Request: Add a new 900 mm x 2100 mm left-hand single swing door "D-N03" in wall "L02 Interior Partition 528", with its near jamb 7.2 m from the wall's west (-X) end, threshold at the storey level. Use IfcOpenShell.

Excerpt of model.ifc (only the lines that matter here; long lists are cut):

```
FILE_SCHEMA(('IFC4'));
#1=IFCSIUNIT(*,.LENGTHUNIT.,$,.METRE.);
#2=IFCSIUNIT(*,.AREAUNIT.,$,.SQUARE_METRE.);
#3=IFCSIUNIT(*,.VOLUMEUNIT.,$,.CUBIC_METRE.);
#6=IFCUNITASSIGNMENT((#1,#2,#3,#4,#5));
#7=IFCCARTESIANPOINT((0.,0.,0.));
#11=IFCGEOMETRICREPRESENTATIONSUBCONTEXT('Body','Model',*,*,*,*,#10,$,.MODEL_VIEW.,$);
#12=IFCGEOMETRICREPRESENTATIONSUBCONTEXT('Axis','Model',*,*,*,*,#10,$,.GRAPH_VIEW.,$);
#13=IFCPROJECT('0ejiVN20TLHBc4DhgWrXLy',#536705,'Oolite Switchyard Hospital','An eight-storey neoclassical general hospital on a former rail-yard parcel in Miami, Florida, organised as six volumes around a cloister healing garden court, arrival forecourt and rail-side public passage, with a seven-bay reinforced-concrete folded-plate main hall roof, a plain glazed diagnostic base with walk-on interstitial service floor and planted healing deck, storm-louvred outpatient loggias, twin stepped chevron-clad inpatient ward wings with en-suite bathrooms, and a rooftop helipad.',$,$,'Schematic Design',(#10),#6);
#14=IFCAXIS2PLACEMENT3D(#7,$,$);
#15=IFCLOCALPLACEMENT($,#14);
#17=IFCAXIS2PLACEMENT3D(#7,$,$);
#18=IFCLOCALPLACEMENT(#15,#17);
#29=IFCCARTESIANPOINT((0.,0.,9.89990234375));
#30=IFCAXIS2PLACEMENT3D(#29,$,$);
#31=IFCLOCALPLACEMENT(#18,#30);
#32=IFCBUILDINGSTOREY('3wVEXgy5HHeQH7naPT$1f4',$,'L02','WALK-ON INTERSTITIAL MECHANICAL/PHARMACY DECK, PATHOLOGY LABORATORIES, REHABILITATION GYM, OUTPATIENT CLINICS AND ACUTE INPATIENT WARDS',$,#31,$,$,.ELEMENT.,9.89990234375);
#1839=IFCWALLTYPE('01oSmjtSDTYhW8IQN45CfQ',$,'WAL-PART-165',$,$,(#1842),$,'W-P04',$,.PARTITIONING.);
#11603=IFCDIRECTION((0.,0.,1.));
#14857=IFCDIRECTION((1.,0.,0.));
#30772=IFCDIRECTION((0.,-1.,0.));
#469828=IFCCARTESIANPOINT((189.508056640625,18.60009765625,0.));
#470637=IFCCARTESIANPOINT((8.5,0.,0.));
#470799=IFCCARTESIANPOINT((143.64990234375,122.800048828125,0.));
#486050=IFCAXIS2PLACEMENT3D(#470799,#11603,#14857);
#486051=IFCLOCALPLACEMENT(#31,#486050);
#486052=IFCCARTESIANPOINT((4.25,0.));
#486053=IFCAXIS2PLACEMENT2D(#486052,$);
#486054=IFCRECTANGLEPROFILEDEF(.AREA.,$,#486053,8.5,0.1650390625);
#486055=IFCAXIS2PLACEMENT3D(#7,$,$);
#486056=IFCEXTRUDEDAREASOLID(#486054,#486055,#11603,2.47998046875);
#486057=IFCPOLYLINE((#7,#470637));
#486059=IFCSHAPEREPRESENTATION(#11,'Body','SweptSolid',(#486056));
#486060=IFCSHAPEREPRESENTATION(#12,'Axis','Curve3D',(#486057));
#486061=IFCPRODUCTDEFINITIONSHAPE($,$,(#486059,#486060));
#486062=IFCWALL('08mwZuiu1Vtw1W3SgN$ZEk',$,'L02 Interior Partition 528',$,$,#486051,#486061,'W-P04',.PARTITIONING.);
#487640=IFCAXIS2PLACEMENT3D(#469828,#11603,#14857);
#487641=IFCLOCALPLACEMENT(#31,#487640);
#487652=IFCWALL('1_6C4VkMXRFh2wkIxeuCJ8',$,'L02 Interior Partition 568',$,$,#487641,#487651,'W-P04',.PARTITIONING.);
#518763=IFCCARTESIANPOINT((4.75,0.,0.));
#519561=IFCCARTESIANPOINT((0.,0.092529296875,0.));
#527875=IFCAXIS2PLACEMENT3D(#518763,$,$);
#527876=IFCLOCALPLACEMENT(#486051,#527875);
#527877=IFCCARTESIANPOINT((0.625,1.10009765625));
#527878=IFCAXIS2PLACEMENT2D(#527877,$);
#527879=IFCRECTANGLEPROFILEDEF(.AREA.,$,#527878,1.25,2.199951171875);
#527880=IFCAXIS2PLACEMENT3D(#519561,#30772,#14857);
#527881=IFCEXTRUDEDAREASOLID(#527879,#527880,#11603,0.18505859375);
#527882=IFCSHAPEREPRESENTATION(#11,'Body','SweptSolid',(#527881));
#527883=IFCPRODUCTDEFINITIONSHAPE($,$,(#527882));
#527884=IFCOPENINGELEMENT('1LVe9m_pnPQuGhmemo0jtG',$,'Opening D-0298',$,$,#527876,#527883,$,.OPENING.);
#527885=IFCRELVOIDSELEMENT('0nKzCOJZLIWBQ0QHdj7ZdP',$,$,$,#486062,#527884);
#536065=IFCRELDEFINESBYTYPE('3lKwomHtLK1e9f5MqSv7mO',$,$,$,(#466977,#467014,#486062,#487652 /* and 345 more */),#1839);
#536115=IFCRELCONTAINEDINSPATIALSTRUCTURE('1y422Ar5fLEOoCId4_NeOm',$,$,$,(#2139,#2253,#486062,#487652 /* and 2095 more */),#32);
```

```python
import numpy as np
import ifcopenshell
import ifcopenshell.api.feature
import ifcopenshell.api.geometry
import ifcopenshell.api.root
import ifcopenshell.api.spatial
import ifcopenshell.geom
import ifcopenshell.util.element
import ifcopenshell.util.placement
import ifcopenshell.util.representation
import ifcopenshell.util.shape
import ifcopenshell.util.unit

model = ifcopenshell.open("model.ifc")
unit_scale = ifcopenshell.util.unit.calculate_unit_scale(model)
settings = ifcopenshell.geom.settings()


def volume(element):
    """Net volume in cubic metres, openings subtracted."""
    shape = ifcopenshell.geom.create_shape(settings, element)
    return ifcopenshell.util.shape.get_volume(shape.geometry)


wall = model.by_id(486062)
storey = ifcopenshell.util.element.get_container(wall, ifc_class="IfcBuildingStorey")
context = ifcopenshell.util.representation.get_context(model, "Model", "Body", "MODEL_VIEW")
before = volume(wall)

width, height, from_end, sill = 0.9, 2.1, 7.2, 0.0  # metres

# The wall runs along its own X axis, and the end named is its -X end.
wall_shape = ifcopenshell.geom.create_shape(settings, wall)
x, y, z = ifcopenshell.util.shape.get_vertices(wall_shape.geometry).T
start = x.min() + from_end
face, thickness = float(y.min()), float(y.max() - y.min())
wall_matrix = ifcopenshell.util.placement.get_local_placement(wall.ObjectPlacement)
level = ifcopenshell.util.placement.get_local_placement(storey.ObjectPlacement)[2, 3]


def in_wall(x, y):
    """Placement at x, y metres in the wall's axes, at sill height."""
    matrix = wall_matrix.copy()
    matrix[:, 3] = wall_matrix @ np.array([x / unit_scale, y / unit_scale, 0.0, 1.0])
    matrix[2, 3] = level + sill / unit_scale
    return matrix


# Opening: a box that overshoots both wall faces by 50 mm.
opening = ifcopenshell.api.root.create_entity(model, ifc_class="IfcOpeningElement", predefined_type="OPENING")
box = ifcopenshell.api.geometry.add_wall_representation(
    model, context=context, length=width, height=height, thickness=thickness + 0.1
)
ifcopenshell.api.geometry.assign_representation(model, product=opening, representation=box)
ifcopenshell.api.geometry.edit_object_placement(model, product=opening, matrix=in_wall(start, face - 0.05), is_si=False)
ifcopenshell.api.feature.add_feature(model, feature=opening, element=wall)

door = ifcopenshell.api.root.create_entity(model, ifc_class="IfcDoor", name="D-N03", predefined_type="DOOR")
door.OverallWidth, door.OverallHeight = width / unit_scale, height / unit_scale
door.OperationType = "SINGLE_SWING_LEFT"
body = ifcopenshell.api.geometry.add_door_representation(
    model,
    context=context,
    overall_width=door.OverallWidth,
    overall_height=door.OverallHeight,
    operation_type="SINGLE_SWING_LEFT",
    lining_properties={"LiningDepth": thickness / unit_scale, "ThresholdDepth": thickness / unit_scale},
)
ifcopenshell.api.geometry.assign_representation(model, product=door, representation=body)
ifcopenshell.api.spatial.assign_container(model, products=[door], relating_structure=storey)
ifcopenshell.api.feature.add_filling(model, opening=opening, element=door)

# The lining spans the wall, so the door starts at the wall face.
ifcopenshell.api.geometry.edit_object_placement(model, product=door, matrix=in_wall(start, face), is_si=False)

after = volume(wall)

print(f"wall volume {before:.3f} -> {after:.3f} m3")

model.write("model_rev.ifc")
```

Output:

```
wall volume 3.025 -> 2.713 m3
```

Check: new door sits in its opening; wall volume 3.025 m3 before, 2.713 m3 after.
